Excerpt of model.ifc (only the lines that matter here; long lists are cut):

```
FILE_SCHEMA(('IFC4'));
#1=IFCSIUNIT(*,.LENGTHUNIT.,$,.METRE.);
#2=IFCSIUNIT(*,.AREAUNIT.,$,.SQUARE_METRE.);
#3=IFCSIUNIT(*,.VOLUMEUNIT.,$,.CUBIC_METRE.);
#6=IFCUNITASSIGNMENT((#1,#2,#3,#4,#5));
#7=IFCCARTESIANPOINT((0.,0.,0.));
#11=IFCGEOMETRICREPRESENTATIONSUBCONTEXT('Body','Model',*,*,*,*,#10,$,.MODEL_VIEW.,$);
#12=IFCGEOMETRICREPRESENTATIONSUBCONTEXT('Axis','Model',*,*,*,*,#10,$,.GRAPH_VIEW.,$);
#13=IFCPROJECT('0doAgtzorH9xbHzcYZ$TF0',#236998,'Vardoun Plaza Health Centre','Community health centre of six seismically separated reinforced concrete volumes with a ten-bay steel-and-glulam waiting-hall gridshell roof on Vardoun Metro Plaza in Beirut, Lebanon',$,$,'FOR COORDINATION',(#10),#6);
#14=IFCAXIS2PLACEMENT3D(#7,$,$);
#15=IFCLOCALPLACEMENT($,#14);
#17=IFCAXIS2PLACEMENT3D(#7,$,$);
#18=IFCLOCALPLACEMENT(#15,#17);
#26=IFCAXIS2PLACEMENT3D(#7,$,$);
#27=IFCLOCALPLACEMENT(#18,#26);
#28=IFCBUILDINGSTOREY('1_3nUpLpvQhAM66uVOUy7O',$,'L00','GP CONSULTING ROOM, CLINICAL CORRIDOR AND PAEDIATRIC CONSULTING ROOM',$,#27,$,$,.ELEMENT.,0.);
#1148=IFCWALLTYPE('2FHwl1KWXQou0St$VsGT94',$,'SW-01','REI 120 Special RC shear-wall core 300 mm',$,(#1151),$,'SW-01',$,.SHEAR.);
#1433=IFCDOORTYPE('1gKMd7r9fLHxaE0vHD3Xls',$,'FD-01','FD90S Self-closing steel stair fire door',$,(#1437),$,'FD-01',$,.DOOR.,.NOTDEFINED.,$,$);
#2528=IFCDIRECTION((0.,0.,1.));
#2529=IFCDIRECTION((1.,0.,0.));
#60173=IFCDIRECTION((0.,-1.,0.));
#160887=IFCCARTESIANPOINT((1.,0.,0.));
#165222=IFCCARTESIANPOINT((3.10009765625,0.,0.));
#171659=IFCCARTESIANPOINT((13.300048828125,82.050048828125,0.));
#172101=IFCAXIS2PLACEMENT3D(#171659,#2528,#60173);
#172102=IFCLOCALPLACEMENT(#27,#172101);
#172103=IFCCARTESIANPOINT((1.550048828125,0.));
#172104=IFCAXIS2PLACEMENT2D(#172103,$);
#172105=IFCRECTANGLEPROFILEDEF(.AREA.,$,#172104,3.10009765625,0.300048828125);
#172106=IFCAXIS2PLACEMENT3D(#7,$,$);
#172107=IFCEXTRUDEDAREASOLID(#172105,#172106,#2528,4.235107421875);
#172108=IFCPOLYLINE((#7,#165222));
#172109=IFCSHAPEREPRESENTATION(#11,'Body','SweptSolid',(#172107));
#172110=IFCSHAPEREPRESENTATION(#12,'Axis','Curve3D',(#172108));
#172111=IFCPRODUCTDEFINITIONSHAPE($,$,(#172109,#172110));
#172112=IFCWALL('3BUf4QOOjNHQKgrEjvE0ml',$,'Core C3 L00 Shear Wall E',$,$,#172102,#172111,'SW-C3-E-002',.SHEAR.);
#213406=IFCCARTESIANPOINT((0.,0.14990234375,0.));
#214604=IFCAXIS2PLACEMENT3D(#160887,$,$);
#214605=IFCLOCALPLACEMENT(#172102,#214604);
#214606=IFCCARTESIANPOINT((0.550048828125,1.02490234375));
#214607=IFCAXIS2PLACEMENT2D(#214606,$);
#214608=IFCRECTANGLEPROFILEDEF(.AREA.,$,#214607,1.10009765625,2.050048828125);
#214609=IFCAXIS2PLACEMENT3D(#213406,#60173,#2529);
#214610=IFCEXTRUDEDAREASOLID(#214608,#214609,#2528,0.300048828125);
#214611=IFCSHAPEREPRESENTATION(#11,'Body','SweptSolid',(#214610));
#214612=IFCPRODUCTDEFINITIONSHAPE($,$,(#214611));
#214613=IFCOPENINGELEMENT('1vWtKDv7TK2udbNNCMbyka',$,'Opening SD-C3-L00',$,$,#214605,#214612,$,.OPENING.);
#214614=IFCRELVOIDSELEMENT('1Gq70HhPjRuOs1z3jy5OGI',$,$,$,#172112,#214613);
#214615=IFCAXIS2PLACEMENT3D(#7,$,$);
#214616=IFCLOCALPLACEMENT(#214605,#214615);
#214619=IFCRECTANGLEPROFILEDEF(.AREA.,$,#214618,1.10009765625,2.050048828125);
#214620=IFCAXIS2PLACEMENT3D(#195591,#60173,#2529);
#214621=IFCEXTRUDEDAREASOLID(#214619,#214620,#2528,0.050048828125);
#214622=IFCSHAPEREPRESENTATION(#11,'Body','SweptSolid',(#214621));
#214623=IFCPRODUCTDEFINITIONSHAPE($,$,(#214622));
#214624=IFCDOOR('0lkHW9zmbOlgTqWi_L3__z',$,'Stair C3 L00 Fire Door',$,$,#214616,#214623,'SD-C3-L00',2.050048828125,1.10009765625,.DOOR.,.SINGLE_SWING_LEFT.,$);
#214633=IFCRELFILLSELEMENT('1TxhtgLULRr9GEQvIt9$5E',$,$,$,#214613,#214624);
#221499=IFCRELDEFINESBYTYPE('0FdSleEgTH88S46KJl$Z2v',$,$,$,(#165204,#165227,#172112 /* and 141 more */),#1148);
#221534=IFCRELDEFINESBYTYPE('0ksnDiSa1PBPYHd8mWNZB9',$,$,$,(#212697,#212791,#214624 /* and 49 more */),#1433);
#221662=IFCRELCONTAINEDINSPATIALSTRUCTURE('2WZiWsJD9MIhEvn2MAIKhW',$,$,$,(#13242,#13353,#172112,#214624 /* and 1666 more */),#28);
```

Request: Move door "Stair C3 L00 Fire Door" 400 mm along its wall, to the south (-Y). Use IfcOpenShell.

```python
import ifcopenshell
import ifcopenshell.api.geometry
import ifcopenshell.util.placement
import ifcopenshell.util.unit

model = ifcopenshell.open("model.ifc")
unit_scale = ifcopenshell.util.unit.calculate_unit_scale(model)

door = model.by_id(214624)
opening = door.FillsVoids[0].RelatingOpeningElement
wall = opening.VoidsElements[0].RelatingBuildingElement

wall_matrix = ifcopenshell.util.placement.get_local_placement(wall.ObjectPlacement)
shift = wall_matrix[:3, 0] * 0.4 / unit_scale
before = ifcopenshell.util.placement.get_local_placement(door.ObjectPlacement)[:3, 3].copy()

# The door is placed relative to its opening, so it follows when the opening moves.
matrix = ifcopenshell.util.placement.get_local_placement(opening.ObjectPlacement)
matrix[:3, 3] += shift
ifcopenshell.api.geometry.edit_object_placement(
    model, product=opening, matrix=matrix, is_si=False, should_transform_children=True
)

after = ifcopenshell.util.placement.get_local_placement(door.ObjectPlacement)[:3, 3]
print("door moved by", (after - before).round(3) + 0.0)

model.write("model_updated.ifc")
```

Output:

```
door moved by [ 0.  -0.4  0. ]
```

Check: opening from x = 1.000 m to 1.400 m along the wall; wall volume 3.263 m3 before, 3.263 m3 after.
